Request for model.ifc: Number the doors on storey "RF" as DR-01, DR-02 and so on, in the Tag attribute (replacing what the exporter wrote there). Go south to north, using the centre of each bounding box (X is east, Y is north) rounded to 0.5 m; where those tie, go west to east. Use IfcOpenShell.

First a look at what the model holds.

```python
import ifcopenshell
import ifcopenshell.util.element
import ifcopenshell.util.placement

model = ifcopenshell.open("model.ifc")
print(model.schema)
storey = next(s for s in model.by_type("IfcBuildingStorey") if s.Name == "RF")
doors = [e for e in ifcopenshell.util.element.get_decomposition(storey) if e.is_a("IfcDoor")]
for e in sorted(doors, key=lambda e: e.id()):
    origin = ifcopenshell.util.placement.get_local_placement(e.ObjectPlacement)[:3, 3]
    print(e.id(), e.Tag, e.Name, origin.round(2) + 0.0, sep=" | ")
```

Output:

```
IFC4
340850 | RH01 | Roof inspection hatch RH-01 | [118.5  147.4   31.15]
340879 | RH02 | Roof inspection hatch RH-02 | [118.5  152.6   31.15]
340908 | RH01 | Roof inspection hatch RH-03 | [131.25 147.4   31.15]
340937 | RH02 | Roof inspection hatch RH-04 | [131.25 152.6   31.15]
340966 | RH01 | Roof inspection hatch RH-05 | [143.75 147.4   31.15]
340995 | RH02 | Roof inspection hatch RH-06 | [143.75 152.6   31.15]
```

```python
import ifcopenshell
import ifcopenshell.geom
import ifcopenshell.util.element
import ifcopenshell.util.shape

model = ifcopenshell.open("model.ifc")
settings = ifcopenshell.geom.settings()
settings.set("use-world-coords", True)


def centre(element):
    shape = ifcopenshell.geom.create_shape(settings, element)
    return ifcopenshell.util.shape.get_bbox_centroid(shape.geometry)


storey = next(s for s in model.by_type("IfcBuildingStorey") if s.Name == "RF")
doors = [e for e in ifcopenshell.util.element.get_decomposition(storey) if e.is_a("IfcDoor")]

# Insertion points can sit at a corner or the storey origin, so sort by the geometry (in metres).
centres = {e: centre(e) for e in doors}
doors.sort(key=lambda e: (round(centres[e][1] / 0.5), centres[e][0]))

for i, e in enumerate(doors, start=1):
    number = f"DR-{i:02d}"
    e.Tag = number
    print(e.id(), number)

model.write("model_updated.ifc")
```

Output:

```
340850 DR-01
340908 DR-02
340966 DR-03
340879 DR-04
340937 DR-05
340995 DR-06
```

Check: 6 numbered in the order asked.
